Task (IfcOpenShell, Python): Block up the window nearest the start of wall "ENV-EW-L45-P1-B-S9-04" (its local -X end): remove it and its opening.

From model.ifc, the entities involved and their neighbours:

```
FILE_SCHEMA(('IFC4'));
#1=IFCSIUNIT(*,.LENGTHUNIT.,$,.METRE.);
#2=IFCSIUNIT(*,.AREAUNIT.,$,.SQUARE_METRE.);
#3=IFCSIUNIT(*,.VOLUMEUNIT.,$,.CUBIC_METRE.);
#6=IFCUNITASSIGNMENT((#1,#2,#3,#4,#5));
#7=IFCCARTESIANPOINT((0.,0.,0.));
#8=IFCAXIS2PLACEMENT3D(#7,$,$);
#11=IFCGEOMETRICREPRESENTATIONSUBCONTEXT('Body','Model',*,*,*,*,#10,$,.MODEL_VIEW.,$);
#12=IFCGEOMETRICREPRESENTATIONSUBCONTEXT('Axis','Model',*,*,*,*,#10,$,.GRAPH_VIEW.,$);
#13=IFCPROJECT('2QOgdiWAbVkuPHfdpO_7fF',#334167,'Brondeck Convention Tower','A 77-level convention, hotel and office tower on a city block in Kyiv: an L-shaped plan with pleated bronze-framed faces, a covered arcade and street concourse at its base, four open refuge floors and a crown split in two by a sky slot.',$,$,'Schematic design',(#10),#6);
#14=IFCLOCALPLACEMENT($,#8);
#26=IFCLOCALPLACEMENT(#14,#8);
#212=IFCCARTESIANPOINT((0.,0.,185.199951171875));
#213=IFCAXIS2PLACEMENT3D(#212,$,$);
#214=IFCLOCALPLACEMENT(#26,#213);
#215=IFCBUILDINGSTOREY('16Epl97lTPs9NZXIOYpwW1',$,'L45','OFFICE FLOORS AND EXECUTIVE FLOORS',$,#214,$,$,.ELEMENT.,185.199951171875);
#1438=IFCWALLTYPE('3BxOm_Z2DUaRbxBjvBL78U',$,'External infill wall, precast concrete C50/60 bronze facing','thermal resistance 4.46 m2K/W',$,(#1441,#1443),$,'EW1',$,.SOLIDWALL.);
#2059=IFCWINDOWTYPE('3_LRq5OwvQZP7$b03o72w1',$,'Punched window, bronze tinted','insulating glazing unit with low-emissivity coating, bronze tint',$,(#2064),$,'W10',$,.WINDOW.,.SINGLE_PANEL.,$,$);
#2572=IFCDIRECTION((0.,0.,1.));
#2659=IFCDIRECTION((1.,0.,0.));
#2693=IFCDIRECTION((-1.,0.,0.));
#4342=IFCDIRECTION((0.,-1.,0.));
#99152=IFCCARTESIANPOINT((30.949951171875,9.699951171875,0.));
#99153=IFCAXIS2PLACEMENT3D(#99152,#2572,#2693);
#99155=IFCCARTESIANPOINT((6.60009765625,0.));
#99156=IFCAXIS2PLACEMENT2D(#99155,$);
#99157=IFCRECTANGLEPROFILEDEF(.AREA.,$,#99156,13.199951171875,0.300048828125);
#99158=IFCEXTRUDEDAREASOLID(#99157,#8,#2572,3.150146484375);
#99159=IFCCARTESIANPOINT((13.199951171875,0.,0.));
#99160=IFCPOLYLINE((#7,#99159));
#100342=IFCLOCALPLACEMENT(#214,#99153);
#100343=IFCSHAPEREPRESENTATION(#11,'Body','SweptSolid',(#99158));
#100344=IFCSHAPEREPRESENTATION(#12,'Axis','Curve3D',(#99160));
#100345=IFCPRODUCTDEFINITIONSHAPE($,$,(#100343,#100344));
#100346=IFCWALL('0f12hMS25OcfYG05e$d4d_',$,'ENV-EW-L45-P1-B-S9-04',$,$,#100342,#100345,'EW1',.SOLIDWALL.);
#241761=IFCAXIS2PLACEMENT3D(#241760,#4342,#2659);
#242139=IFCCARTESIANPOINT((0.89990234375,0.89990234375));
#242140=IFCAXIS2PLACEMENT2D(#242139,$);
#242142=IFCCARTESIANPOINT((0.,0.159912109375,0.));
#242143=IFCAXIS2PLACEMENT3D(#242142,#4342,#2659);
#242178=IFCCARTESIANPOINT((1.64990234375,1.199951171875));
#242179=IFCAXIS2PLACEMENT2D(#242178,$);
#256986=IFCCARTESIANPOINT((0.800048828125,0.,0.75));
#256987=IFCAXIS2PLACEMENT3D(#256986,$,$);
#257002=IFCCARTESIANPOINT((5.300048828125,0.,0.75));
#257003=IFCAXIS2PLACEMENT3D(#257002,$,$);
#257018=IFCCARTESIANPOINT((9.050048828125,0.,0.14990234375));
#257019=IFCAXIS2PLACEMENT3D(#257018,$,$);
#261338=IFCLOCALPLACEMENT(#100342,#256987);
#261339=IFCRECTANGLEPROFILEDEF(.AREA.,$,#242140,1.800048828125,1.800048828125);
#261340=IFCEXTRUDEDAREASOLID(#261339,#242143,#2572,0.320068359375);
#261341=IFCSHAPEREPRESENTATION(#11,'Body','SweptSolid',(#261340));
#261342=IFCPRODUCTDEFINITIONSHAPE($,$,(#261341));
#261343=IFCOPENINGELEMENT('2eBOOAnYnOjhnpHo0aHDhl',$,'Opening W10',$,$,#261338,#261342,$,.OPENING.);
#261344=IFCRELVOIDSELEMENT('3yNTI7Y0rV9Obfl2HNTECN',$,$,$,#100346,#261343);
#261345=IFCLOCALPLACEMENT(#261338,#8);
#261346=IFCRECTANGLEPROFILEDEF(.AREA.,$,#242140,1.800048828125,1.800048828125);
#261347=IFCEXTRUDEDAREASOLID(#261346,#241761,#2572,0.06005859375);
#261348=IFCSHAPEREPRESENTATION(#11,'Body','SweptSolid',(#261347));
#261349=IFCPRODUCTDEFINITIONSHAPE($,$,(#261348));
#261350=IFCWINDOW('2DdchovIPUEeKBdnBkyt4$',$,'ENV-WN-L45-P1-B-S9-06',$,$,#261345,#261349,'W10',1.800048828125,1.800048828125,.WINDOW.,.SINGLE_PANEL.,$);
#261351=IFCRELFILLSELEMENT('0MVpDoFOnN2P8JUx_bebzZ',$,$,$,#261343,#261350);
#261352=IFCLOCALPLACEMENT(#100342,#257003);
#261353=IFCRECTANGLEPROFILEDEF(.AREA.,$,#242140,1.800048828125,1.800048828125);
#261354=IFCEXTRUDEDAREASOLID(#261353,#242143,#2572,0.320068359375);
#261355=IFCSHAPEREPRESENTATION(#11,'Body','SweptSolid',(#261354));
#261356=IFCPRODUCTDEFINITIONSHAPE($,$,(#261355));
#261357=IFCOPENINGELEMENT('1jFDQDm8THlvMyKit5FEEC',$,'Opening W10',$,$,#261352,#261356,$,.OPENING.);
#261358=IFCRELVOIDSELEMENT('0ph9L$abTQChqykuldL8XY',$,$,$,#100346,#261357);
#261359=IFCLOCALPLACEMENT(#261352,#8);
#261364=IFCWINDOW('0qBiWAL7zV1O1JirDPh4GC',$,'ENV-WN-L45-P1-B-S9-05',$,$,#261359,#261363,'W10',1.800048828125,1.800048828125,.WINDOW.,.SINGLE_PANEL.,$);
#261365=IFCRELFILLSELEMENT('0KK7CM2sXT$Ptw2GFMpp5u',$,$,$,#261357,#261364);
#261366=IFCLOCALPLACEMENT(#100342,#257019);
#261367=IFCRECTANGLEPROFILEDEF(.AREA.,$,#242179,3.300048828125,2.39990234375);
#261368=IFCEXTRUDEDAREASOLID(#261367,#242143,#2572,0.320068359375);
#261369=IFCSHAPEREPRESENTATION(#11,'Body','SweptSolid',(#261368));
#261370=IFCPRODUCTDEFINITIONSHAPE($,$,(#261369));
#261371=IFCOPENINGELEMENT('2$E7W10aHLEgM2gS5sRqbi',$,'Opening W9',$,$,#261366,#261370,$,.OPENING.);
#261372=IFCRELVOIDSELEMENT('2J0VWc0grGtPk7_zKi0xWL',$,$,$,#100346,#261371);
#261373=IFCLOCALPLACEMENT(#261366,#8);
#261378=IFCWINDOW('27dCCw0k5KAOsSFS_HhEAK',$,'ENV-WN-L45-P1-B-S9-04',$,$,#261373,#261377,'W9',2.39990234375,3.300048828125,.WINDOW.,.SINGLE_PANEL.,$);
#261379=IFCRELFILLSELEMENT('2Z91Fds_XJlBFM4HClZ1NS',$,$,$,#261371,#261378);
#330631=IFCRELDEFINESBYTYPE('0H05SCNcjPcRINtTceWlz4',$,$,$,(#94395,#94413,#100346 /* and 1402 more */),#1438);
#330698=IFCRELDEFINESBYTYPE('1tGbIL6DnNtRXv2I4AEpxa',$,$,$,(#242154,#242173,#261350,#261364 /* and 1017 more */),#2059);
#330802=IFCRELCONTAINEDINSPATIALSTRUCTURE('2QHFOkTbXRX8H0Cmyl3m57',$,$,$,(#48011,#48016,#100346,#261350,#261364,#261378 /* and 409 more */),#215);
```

```python
import ifcopenshell
import ifcopenshell.api.feature
import ifcopenshell.api.root
import ifcopenshell.geom
import ifcopenshell.util.shape

model = ifcopenshell.open("model.ifc")
settings = ifcopenshell.geom.settings()


def volume(element):
    """Net volume in cubic metres, openings subtracted."""
    shape = ifcopenshell.geom.create_shape(settings, element)
    return ifcopenshell.util.shape.get_volume(shape.geometry)


window = model.by_guid("2DdchovIPUEeKBdnBkyt4$")
opening = window.FillsVoids[0].RelatingOpeningElement
wall = opening.VoidsElements[0].RelatingBuildingElement
before = volume(wall)

ifcopenshell.api.root.remove_product(model, product=window)
ifcopenshell.api.feature.remove_feature(model, feature=opening)

after = volume(wall)

print(f"wall volume {before:.3f} -> {after:.3f} m3")

model.write("model_v2.ifc")
```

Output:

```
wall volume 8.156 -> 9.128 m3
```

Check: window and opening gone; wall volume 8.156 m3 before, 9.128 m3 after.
